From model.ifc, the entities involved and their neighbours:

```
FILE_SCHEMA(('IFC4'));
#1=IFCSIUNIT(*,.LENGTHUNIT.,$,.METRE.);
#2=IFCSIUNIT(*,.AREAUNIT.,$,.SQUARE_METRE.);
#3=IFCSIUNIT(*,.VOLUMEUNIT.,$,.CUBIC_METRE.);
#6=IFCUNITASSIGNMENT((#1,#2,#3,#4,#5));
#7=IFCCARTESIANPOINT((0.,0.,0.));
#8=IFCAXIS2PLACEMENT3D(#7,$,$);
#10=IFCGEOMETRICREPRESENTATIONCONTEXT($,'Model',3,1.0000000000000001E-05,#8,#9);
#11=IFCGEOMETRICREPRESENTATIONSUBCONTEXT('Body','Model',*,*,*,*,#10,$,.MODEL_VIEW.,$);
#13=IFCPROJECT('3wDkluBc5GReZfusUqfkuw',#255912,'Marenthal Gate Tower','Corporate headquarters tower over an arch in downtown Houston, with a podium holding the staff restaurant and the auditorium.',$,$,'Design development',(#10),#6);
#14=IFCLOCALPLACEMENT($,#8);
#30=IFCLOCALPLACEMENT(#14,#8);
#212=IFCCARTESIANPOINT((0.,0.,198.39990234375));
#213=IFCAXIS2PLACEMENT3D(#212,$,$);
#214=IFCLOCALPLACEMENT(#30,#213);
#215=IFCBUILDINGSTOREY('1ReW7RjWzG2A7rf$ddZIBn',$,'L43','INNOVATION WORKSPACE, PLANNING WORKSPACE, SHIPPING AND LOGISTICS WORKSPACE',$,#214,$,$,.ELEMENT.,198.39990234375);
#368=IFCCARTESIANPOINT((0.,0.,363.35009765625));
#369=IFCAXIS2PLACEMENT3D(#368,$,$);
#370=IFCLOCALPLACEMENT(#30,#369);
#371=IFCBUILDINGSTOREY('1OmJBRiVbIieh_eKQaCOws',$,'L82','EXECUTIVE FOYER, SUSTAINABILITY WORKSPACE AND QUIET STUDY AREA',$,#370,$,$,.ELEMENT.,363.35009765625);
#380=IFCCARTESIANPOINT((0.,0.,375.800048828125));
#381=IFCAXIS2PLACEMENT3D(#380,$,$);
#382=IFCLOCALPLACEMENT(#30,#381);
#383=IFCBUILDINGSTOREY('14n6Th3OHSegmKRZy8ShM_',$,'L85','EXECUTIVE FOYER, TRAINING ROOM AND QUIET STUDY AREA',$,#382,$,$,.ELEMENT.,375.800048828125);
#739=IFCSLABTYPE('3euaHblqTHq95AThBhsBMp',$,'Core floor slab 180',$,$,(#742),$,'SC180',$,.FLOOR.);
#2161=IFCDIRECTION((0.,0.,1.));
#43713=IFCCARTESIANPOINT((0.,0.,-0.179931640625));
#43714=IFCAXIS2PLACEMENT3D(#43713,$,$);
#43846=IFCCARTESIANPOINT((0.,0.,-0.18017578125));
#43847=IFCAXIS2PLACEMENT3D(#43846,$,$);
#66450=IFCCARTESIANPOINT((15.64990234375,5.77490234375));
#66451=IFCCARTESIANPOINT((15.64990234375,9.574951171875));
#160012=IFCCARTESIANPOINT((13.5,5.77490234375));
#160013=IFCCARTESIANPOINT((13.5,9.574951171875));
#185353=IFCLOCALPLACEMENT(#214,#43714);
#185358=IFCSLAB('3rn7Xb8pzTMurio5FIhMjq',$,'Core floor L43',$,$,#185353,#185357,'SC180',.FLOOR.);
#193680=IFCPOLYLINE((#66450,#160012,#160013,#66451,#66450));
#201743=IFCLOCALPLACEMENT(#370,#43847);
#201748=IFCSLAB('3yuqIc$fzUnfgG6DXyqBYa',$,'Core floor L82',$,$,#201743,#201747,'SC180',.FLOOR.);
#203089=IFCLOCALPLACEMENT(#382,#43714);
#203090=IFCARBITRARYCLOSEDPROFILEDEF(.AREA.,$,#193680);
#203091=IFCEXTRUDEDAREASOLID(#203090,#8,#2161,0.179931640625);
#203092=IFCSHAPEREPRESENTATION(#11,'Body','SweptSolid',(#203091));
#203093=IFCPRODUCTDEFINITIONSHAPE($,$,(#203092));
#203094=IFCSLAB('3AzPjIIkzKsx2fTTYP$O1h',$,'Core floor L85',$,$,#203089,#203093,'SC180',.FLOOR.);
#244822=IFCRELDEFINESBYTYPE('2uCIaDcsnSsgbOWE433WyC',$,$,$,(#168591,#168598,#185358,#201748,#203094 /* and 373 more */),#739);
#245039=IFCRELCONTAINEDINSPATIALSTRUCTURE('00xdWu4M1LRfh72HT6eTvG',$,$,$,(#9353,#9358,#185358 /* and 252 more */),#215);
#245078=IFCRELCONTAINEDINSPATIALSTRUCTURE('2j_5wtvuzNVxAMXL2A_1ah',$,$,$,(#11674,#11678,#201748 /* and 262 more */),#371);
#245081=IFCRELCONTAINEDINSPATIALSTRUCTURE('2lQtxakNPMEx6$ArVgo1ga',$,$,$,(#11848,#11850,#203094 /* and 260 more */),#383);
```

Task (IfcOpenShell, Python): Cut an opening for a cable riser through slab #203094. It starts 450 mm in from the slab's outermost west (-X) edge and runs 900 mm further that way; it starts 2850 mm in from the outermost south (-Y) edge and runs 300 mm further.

```python
import numpy as np
import ifcopenshell
import ifcopenshell.api.feature
import ifcopenshell.api.geometry
import ifcopenshell.api.root
import ifcopenshell.geom
import ifcopenshell.util.placement
import ifcopenshell.util.representation
import ifcopenshell.util.shape
import ifcopenshell.util.unit

model = ifcopenshell.open("model.ifc")
unit_scale = ifcopenshell.util.unit.calculate_unit_scale(model)
settings = ifcopenshell.geom.settings()


def volume(element):
    """Net volume in cubic metres, openings subtracted."""
    shape = ifcopenshell.geom.create_shape(settings, element)
    return ifcopenshell.util.shape.get_volume(shape.geometry)


slab = model.by_guid("3AzPjIIkzKsx2fTTYP$O1h")
before = volume(slab)

# Extent in the slab's own axes, in metres. The edges named are its -X and -Y sides.
slab_shape = ifcopenshell.geom.create_shape(settings, slab)
vertices = ifcopenshell.util.shape.get_vertices(slab_shape.geometry)
x_min, y_min, bottom = vertices.min(axis=0)
top = vertices[:, 2].max()

opening = ifcopenshell.api.root.create_entity(model, ifc_class="IfcOpeningElement", name="Cable riser opening", predefined_type="OPENING")
context = ifcopenshell.util.representation.get_context(model, "Model", "Body", "MODEL_VIEW")
width, depth = 0.9, 0.3
outline = [(0.0, 0.0), (width, 0.0), (width, depth), (0.0, depth), (0.0, 0.0)]
# Overshoot both faces by 50 mm so the cut is clean.
shape = ifcopenshell.api.geometry.add_slab_representation(
    model, context=context, depth=top - bottom + 0.1, polyline=outline
)
ifcopenshell.api.geometry.assign_representation(model, product=opening, representation=shape)

matrix = ifcopenshell.util.placement.get_local_placement(slab.ObjectPlacement)
matrix[:, 3] = matrix @ np.append(np.array([x_min + 0.45, y_min + 2.85, bottom - 0.05]) / unit_scale, 1.0)
ifcopenshell.api.geometry.edit_object_placement(model, product=opening, matrix=matrix, is_si=False)
ifcopenshell.api.feature.add_feature(model, feature=opening, element=slab)

after = volume(slab)

print(f"slab volume {before:.3f} -> {after:.3f} m3")

model.write("model-out.ifc")
```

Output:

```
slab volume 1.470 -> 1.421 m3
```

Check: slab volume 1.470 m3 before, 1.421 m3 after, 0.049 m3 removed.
